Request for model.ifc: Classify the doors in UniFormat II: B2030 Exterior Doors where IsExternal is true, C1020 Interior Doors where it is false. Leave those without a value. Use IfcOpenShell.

First a look at what the model holds.

```python
import ifcopenshell
import ifcopenshell.util.element

model = ifcopenshell.open("model.ifc")
print(model.schema)
print("classifications:", [c.Name for c in model.by_type("IfcClassification")])
values = [ifcopenshell.util.element.get_pset(e, "Pset_DoorCommon", "IsExternal") for e in model.by_type("IfcDoor")]
for value in (True, False, None):
    print("IsExternal", value, values.count(value))
```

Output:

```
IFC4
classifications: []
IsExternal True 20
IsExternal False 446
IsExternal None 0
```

```python
import ifcopenshell
import ifcopenshell.api.classification
import ifcopenshell.util.element

model = ifcopenshell.open("model.ifc")

system = ifcopenshell.api.classification.add_classification(model, classification="UniFormat II")

doors = model.by_type("IfcDoor")
external = {e: ifcopenshell.util.element.get_pset(e, "Pset_DoorCommon", "IsExternal") for e in doors}
for flag, code, name in ((True, "B2030", "Exterior Doors"), (False, "C1020", "Interior Doors")):
    products = [e for e in doors if external[e] is flag]
    ifcopenshell.api.classification.add_reference(
        model, products=products, classification=system, identification=code, name=name
    )
    print(code, len(products))

model.write("model_edited.ifc")
```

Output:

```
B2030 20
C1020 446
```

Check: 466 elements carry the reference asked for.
